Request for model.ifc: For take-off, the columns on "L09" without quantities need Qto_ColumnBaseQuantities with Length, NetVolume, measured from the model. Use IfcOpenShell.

First a look at what the model holds.

```python
import ifcopenshell
import ifcopenshell.util.element
import ifcopenshell.util.unit

model = ifcopenshell.open("model.ifc")
print(model.schema)
for unit_type in ("LENGTHUNIT", "AREAUNIT", "VOLUMEUNIT"):
    print(unit_type, ifcopenshell.util.unit.calculate_unit_scale(model, unit_type))
storey = next(s for s in model.by_type("IfcBuildingStorey") if s.Name == "L09")
columns = [e for e in ifcopenshell.util.element.get_decomposition(storey) if e.is_a("IfcColumn")]
for e in sorted(columns, key=lambda e: e.id()):
    print(e.id(), e.is_a(), e.Name, list(ifcopenshell.util.element.get_psets(e, qtos_only=True)), sep=" | ")
```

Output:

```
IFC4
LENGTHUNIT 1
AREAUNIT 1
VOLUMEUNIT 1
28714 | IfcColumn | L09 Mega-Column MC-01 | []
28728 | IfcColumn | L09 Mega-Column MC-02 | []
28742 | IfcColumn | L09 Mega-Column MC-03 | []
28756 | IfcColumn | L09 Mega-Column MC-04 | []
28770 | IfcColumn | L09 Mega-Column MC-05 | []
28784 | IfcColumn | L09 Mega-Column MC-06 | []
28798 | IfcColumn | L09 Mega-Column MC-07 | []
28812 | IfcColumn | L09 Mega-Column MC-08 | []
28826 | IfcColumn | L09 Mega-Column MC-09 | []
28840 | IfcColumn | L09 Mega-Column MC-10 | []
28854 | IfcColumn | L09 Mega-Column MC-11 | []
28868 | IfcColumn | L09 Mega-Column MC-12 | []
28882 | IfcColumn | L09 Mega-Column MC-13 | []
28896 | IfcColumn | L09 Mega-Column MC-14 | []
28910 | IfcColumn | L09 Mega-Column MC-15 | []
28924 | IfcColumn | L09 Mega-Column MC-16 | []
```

```python
import ifcopenshell
import ifcopenshell.api.pset
import ifcopenshell.geom
import ifcopenshell.util.element
import ifcopenshell.util.shape
import ifcopenshell.util.unit

model = ifcopenshell.open("model.ifc")
unit_scale = ifcopenshell.util.unit.calculate_unit_scale(model)
volume_scale = ifcopenshell.util.unit.calculate_unit_scale(model, "VOLUMEUNIT")
settings = ifcopenshell.geom.settings()

storey = next(s for s in model.by_type("IfcBuildingStorey") if s.Name == "L09")
columns = [e for e in ifcopenshell.util.element.get_decomposition(storey) if e.is_a("IfcColumn")]

for e in sorted(columns, key=lambda e: e.id()):
    if ifcopenshell.util.element.get_psets(e, qtos_only=True, should_inherit=False):
        continue
    # Geometry comes back in metres, in the element's own axes.
    shape = ifcopenshell.geom.create_shape(settings, e)
    values = {
        "Length": ifcopenshell.util.shape.get_z(shape.geometry) / unit_scale,
        "NetVolume": ifcopenshell.util.shape.get_volume(shape.geometry) / volume_scale,
    }
    qto = ifcopenshell.api.pset.add_qto(model, product=e, name="Qto_ColumnBaseQuantities")
    ifcopenshell.api.pset.edit_qto(model, qto=qto, properties=values)
    print(e.id(), {k: round(v, 3) for k, v in values.items()})

model.write("model-out.ifc")
```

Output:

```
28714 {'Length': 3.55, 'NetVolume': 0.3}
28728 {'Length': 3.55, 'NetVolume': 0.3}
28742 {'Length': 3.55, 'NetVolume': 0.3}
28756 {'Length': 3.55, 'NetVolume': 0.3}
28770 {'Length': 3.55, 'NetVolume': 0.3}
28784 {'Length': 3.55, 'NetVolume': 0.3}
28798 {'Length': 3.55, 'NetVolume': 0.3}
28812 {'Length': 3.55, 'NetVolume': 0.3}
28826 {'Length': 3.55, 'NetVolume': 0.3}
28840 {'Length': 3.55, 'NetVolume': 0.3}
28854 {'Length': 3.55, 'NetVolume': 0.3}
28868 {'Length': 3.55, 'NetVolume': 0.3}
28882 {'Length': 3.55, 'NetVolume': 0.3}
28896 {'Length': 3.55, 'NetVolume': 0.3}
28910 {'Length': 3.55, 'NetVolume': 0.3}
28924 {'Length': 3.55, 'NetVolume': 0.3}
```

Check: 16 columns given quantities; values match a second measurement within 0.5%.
